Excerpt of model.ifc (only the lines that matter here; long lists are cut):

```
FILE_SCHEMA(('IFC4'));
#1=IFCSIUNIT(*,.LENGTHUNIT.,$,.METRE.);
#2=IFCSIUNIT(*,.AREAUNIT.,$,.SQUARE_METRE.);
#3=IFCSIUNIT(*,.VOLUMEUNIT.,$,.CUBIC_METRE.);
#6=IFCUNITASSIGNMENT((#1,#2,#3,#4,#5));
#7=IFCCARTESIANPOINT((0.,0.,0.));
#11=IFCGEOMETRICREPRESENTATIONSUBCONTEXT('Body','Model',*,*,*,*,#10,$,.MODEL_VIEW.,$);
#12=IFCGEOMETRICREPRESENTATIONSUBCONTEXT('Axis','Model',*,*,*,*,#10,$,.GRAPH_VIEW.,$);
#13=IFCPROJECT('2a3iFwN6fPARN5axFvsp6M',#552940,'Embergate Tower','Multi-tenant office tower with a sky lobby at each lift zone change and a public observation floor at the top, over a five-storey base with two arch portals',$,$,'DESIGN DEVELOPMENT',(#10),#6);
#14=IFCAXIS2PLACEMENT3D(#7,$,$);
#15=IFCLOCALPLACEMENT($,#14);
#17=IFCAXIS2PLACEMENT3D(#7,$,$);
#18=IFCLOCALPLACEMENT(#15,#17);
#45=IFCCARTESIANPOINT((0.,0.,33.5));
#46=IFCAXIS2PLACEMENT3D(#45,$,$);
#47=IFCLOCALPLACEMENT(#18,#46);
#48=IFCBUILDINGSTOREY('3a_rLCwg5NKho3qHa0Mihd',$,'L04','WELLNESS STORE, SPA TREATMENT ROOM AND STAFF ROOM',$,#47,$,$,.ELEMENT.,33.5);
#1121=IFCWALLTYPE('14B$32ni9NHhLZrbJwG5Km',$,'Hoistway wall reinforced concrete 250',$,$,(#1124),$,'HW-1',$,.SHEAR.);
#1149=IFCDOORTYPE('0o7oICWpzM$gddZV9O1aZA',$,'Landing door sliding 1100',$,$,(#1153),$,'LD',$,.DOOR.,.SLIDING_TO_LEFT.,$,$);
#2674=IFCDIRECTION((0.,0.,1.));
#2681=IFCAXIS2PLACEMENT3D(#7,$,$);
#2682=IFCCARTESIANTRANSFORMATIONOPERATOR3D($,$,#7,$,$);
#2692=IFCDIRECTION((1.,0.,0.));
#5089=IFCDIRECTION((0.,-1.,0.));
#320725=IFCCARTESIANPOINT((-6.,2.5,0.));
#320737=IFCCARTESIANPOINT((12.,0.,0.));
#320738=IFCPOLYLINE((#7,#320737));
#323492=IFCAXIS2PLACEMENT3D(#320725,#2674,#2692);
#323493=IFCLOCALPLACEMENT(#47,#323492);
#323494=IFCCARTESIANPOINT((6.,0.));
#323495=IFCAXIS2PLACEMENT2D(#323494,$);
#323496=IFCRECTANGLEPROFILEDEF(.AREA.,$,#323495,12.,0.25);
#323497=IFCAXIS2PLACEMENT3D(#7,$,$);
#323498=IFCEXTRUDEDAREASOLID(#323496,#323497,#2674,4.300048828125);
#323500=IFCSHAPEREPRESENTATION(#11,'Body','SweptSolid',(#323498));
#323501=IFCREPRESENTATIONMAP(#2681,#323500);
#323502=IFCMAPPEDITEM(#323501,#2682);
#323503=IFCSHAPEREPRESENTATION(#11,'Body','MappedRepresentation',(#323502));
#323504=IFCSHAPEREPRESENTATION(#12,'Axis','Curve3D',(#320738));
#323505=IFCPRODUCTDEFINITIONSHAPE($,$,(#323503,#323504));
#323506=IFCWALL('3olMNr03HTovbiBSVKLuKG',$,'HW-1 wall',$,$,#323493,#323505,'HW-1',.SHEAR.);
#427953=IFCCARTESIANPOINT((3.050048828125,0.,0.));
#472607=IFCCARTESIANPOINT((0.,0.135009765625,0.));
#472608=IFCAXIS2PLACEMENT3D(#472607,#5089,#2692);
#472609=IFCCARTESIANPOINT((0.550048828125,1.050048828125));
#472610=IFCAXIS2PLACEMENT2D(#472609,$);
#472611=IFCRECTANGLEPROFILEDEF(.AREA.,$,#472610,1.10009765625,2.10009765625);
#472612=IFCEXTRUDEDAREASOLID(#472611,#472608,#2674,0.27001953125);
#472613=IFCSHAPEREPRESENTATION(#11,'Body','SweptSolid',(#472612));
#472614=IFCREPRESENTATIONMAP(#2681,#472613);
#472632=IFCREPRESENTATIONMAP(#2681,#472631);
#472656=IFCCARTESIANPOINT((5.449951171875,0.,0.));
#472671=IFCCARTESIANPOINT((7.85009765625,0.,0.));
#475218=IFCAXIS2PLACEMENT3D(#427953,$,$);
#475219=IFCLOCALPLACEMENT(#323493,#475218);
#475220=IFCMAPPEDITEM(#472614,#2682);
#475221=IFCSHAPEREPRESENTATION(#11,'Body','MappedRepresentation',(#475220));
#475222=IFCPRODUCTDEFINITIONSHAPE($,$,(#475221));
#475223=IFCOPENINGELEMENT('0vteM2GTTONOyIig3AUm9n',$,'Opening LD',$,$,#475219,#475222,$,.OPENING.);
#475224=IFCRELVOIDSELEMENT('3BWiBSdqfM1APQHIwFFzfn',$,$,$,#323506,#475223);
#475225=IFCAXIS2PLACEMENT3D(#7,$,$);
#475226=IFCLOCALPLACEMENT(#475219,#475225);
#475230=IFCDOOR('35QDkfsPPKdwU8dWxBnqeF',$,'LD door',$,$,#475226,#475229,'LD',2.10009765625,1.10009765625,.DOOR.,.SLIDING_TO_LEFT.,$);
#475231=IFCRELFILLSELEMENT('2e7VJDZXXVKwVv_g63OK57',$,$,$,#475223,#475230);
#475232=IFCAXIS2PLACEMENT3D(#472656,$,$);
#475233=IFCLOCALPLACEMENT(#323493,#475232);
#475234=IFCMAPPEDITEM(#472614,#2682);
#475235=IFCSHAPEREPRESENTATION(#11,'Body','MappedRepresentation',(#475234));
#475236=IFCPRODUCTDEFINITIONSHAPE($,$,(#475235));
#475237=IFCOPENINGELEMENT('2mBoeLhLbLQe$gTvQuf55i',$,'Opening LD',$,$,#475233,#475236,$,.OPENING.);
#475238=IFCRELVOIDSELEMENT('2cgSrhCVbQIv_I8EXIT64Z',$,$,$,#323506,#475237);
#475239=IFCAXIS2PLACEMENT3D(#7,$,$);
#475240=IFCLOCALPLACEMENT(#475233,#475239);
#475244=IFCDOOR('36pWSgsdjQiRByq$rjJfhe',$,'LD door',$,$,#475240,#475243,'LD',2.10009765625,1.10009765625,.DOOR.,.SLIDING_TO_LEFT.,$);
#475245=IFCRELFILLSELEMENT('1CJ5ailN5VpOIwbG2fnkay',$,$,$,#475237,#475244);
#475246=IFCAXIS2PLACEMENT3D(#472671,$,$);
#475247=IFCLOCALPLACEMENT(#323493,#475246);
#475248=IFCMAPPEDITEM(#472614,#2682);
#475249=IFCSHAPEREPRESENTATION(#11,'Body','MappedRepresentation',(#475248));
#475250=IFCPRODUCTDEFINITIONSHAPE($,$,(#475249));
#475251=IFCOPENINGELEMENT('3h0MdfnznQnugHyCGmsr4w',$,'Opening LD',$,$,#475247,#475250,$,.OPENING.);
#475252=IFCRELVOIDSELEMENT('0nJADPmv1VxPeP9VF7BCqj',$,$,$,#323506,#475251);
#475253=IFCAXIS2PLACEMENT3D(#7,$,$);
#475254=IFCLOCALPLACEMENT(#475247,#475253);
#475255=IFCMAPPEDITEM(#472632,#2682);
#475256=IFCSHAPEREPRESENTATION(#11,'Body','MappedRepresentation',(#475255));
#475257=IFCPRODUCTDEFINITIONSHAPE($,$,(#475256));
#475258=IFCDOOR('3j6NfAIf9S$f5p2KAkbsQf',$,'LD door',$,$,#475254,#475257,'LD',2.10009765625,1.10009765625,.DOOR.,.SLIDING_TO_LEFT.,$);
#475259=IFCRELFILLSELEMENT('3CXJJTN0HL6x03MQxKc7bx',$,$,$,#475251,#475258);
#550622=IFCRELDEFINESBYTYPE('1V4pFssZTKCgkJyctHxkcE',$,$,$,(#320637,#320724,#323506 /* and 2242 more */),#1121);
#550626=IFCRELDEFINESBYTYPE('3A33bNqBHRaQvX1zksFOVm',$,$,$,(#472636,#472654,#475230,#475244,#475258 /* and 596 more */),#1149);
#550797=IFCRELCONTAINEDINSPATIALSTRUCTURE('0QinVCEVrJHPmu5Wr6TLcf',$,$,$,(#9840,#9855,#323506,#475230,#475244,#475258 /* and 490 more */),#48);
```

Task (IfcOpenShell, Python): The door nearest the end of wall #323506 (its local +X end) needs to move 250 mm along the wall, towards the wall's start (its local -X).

```python
import ifcopenshell
import ifcopenshell.api.geometry
import ifcopenshell.util.placement
import ifcopenshell.util.unit

model = ifcopenshell.open("model.ifc")
unit_scale = ifcopenshell.util.unit.calculate_unit_scale(model)

door = model.by_guid("3j6NfAIf9S$f5p2KAkbsQf")
opening = door.FillsVoids[0].RelatingOpeningElement
wall = opening.VoidsElements[0].RelatingBuildingElement

wall_matrix = ifcopenshell.util.placement.get_local_placement(wall.ObjectPlacement)
shift = wall_matrix[:3, 0] * -0.25 / unit_scale
before = ifcopenshell.util.placement.get_local_placement(door.ObjectPlacement)[:3, 3].copy()

# The door is placed relative to its opening, so it follows when the opening moves.
matrix = ifcopenshell.util.placement.get_local_placement(opening.ObjectPlacement)
matrix[:3, 3] += shift
ifcopenshell.api.geometry.edit_object_placement(
    model, product=opening, matrix=matrix, is_si=False, should_transform_children=True
)

after = ifcopenshell.util.placement.get_local_placement(door.ObjectPlacement)[:3, 3]
print("door moved by", (after - before).round(3) + 0.0)

model.write("model_edited.ifc")
```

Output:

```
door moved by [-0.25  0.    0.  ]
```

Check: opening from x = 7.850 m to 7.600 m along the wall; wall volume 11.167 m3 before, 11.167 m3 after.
